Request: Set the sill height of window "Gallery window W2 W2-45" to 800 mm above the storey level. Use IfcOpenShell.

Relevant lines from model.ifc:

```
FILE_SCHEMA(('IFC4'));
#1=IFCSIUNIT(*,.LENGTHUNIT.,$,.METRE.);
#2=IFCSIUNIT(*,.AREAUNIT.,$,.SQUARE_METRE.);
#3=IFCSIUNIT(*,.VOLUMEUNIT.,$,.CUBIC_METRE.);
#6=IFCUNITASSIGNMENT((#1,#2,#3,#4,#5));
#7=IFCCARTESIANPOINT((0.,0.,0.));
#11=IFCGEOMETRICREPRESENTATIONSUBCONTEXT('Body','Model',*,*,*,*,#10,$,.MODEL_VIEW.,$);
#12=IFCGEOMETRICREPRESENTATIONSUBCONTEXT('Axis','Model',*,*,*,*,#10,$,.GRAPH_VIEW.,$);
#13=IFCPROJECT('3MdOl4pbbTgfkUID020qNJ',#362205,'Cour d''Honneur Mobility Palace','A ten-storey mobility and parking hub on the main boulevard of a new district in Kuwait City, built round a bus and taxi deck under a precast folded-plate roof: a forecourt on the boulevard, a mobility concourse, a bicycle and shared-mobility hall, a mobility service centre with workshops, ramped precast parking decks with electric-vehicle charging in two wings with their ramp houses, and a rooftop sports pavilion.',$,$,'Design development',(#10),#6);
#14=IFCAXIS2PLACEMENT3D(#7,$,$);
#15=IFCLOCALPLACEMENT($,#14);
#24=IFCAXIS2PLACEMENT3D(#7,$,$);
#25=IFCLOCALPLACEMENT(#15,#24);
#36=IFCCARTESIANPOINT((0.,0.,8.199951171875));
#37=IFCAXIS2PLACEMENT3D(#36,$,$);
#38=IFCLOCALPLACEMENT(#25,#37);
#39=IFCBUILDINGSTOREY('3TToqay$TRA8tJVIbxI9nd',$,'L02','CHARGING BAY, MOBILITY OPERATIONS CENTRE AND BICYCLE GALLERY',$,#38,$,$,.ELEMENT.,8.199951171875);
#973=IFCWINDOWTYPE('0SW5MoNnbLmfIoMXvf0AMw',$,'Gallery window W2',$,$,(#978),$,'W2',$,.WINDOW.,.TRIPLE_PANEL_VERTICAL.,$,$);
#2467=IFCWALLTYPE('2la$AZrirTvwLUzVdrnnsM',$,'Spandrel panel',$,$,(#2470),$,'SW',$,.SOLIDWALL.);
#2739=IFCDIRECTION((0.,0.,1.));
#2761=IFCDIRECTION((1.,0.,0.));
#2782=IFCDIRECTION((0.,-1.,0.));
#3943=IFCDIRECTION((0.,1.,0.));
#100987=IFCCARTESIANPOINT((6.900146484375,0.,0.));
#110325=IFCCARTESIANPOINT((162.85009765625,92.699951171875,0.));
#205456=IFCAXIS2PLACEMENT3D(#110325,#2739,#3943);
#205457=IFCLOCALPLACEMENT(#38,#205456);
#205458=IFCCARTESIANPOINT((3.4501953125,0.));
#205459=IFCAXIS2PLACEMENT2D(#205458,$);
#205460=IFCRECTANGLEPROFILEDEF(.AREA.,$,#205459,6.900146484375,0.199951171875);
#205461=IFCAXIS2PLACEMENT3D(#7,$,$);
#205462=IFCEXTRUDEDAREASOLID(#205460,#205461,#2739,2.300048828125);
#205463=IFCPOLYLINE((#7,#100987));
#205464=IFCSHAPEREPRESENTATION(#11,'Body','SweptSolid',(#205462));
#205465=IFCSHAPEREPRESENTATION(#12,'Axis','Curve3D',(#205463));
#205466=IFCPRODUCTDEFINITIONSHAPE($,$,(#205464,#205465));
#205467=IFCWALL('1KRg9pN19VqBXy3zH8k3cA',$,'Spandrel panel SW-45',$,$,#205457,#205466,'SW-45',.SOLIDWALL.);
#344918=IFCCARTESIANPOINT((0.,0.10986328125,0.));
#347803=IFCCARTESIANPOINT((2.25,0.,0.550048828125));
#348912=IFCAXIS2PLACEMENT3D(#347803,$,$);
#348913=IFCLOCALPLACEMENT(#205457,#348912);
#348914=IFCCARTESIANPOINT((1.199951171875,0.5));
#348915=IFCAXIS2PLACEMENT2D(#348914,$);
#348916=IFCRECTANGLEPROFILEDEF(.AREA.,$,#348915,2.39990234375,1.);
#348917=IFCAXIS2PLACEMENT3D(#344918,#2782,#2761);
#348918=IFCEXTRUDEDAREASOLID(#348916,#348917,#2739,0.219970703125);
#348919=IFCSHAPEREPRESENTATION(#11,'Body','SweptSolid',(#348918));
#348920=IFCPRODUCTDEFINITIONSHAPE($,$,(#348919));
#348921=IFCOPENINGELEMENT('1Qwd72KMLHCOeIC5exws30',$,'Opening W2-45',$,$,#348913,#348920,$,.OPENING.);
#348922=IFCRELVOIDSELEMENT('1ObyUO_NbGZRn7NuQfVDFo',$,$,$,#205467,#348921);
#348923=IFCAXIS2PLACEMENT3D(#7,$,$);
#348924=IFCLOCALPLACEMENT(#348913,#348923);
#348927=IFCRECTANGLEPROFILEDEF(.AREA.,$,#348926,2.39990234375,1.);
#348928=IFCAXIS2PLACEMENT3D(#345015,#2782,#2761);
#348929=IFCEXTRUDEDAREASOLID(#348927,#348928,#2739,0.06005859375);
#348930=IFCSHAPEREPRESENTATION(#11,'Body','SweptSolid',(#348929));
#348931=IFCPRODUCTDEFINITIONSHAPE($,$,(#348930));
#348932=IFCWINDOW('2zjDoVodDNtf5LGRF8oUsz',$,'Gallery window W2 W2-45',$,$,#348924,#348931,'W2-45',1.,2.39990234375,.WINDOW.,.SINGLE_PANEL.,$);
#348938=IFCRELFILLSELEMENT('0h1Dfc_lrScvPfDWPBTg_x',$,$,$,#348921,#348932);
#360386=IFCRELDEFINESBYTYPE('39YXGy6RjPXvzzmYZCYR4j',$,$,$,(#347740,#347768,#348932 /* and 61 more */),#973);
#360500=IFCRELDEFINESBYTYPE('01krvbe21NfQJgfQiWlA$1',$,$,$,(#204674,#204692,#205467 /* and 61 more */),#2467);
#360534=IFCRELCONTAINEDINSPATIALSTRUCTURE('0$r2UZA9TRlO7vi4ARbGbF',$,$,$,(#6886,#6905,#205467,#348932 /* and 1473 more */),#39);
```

```python
import numpy as np
import ifcopenshell
import ifcopenshell.api.geometry
import ifcopenshell.geom
import ifcopenshell.util.element
import ifcopenshell.util.placement
import ifcopenshell.util.shape
import ifcopenshell.util.unit

model = ifcopenshell.open("model.ifc")
unit_scale = ifcopenshell.util.unit.calculate_unit_scale(model)

window = model.by_guid("2zjDoVodDNtf5LGRF8oUsz")
opening = window.FillsVoids[0].RelatingOpeningElement
storey = ifcopenshell.util.element.get_container(window, ifc_class="IfcBuildingStorey")
level = ifcopenshell.util.placement.get_local_placement(storey.ObjectPlacement)[2, 3]

# The opening's origin need not be at the sill, so measure its lowest point.
shape = ifcopenshell.geom.create_shape(ifcopenshell.geom.settings(), opening)
bottom = ifcopenshell.util.shape.get_shape_bottom_elevation(shape, shape.geometry) / unit_scale
dz = level + 0.8 - bottom

shift = np.array([0.0, 0.0, dz])
# The window is placed relative to its opening, so it follows when the opening moves.
matrix = ifcopenshell.util.placement.get_local_placement(opening.ObjectPlacement)
matrix[:3, 3] += shift
ifcopenshell.api.geometry.edit_object_placement(
    model, product=opening, matrix=matrix, is_si=False, should_transform_children=True
)

print(f"moved by {dz * unit_scale:+.3f} m")

model.write("model_rev.ifc")
```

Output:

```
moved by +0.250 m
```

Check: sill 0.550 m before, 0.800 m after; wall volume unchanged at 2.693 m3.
